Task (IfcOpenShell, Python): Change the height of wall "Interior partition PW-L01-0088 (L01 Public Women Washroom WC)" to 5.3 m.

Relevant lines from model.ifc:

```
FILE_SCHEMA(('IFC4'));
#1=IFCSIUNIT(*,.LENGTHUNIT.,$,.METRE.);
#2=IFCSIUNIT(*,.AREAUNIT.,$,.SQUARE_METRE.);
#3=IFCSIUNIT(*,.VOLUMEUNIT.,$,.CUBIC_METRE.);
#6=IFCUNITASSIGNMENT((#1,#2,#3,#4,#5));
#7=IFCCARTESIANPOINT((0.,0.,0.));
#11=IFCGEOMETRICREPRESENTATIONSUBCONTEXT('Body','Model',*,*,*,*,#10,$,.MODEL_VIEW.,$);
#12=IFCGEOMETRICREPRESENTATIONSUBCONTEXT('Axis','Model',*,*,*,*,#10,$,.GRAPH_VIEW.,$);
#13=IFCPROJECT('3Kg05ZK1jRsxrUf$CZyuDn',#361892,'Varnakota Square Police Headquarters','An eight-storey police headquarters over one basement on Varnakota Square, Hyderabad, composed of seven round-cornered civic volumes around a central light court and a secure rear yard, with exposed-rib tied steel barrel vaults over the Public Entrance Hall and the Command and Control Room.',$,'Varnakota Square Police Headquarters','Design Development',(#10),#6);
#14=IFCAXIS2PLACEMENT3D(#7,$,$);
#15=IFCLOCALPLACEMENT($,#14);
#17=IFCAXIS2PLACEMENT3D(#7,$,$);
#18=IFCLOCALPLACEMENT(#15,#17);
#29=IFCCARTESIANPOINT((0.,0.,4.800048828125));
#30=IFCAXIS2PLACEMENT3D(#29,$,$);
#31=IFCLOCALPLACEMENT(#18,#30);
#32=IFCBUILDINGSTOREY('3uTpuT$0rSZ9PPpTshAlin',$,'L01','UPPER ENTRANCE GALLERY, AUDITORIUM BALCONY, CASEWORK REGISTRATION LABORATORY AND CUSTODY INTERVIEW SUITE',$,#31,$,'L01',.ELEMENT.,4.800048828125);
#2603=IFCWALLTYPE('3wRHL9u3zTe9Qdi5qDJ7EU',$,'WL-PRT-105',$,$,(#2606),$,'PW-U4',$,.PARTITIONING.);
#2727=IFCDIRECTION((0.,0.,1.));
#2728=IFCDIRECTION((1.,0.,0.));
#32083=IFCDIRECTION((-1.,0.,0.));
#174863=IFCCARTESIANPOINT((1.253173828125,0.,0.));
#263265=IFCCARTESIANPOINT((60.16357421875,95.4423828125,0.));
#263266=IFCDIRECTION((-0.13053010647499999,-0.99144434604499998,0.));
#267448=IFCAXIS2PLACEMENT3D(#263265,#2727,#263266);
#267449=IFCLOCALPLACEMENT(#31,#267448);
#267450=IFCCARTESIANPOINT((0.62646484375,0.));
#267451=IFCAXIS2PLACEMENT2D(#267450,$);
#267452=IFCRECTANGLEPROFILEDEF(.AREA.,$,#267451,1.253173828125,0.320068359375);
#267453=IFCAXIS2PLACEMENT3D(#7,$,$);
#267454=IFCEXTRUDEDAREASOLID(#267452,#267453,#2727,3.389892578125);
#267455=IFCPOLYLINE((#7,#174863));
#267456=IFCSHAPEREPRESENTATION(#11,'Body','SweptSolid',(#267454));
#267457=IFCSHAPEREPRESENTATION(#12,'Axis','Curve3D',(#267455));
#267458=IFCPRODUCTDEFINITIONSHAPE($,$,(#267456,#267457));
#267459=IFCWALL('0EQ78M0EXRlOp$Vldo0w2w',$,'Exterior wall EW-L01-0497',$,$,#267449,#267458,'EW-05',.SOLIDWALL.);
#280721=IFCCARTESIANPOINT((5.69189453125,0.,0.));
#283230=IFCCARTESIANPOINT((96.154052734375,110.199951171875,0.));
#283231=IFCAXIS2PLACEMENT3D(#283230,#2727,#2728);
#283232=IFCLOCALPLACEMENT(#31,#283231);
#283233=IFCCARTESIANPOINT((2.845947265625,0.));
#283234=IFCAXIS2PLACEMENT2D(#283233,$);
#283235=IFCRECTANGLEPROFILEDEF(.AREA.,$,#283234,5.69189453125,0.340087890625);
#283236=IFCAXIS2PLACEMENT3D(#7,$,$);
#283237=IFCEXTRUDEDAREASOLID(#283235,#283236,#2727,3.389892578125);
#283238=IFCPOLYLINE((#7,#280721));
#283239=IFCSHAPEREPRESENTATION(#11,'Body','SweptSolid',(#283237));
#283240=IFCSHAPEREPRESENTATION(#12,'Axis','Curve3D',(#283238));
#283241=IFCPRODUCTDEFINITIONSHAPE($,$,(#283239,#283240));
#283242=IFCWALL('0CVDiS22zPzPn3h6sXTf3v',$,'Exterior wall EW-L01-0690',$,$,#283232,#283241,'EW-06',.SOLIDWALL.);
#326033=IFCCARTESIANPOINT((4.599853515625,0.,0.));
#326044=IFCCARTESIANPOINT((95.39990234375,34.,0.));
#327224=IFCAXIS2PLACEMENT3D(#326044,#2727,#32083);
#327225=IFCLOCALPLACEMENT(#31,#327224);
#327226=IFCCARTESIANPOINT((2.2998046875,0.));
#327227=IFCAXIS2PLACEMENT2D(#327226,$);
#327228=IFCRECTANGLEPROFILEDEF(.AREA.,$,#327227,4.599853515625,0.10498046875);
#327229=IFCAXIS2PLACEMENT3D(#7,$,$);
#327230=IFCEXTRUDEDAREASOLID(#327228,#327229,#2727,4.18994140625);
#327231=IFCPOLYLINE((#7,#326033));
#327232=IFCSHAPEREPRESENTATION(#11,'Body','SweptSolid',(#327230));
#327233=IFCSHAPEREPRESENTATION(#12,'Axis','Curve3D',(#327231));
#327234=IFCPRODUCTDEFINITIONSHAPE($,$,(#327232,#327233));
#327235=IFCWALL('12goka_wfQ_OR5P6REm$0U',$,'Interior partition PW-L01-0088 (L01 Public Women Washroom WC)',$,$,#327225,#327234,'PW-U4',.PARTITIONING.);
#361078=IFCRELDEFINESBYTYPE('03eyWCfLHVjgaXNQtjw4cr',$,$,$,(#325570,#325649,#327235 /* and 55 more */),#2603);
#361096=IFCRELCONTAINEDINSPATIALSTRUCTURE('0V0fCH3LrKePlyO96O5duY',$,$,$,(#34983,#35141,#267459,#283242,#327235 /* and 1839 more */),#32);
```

```python
import ifcopenshell
import ifcopenshell.geom
import ifcopenshell.util.representation
import ifcopenshell.util.shape
import ifcopenshell.util.unit

model = ifcopenshell.open("model.ifc")
unit_scale = ifcopenshell.util.unit.calculate_unit_scale(model)
settings = ifcopenshell.geom.settings()


def volume(element):
    """Net volume in cubic metres, openings subtracted."""
    shape = ifcopenshell.geom.create_shape(settings, element)
    return ifcopenshell.util.shape.get_volume(shape.geometry)


wall = model.by_guid("12goka_wfQ_OR5P6REm$0U")
before = volume(wall)

body = ifcopenshell.util.representation.get_representation(wall, "Model", "Body")
solid = body.Items[0]
old_height = solid.Depth
solid.Depth = 5.3 / unit_scale
after = volume(wall)

print(f"height {old_height:g} -> {solid.Depth:g}, volume {before:.3f} -> {after:.3f} m3")

model.write("model_rev.ifc")
```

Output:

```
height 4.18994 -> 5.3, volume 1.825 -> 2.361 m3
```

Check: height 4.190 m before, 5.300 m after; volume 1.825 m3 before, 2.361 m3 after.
